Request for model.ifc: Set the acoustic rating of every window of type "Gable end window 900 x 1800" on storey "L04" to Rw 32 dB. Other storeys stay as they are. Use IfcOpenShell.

First a look at what the model holds.

```python
import ifcopenshell
import ifcopenshell.util.element

model = ifcopenshell.open("model.ifc")
print(model.schema)
storey = next(s for s in model.by_type("IfcBuildingStorey") if s.Name == "L04")
windows = [e for e in ifcopenshell.util.element.get_decomposition(storey) if e.is_a("IfcWindow")]
seen = {}
for e in windows:
    element_type = ifcopenshell.util.element.get_type(e)
    key = (element_type.Name if element_type != e and element_type else None, ifcopenshell.util.element.get_pset(e, "Pset_WindowCommon", "AcousticRating"))
    seen[key] = seen.get(key, 0) + 1
for (name, value), count in sorted(seen.items(), key=str):
    print(count, "x", name, "|", value)
```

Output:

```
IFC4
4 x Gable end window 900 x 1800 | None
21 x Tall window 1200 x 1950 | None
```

```python
import ifcopenshell
import ifcopenshell.api.pset
import ifcopenshell.util.element

model = ifcopenshell.open("model.ifc")

storey = next(s for s in model.by_type("IfcBuildingStorey") if s.Name == "L04")
windows = [e for e in ifcopenshell.util.element.get_decomposition(storey) if e.is_a("IfcWindow")]

count = 0
for e in windows:
    element_type = ifcopenshell.util.element.get_type(e)
    if element_type in (None, e) or element_type.Name != "Gable end window 900 x 1800":
        continue
    # add_pset returns the element's existing set when there is one.
    pset = ifcopenshell.api.pset.add_pset(model, product=e, name="Pset_WindowCommon")
    ifcopenshell.api.pset.edit_pset(model, pset=pset, properties={"AcousticRating": "Rw 32 dB"})
    count += 1

print(count, "windows updated")

model.write("model_v2.ifc")
```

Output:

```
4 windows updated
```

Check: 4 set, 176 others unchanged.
